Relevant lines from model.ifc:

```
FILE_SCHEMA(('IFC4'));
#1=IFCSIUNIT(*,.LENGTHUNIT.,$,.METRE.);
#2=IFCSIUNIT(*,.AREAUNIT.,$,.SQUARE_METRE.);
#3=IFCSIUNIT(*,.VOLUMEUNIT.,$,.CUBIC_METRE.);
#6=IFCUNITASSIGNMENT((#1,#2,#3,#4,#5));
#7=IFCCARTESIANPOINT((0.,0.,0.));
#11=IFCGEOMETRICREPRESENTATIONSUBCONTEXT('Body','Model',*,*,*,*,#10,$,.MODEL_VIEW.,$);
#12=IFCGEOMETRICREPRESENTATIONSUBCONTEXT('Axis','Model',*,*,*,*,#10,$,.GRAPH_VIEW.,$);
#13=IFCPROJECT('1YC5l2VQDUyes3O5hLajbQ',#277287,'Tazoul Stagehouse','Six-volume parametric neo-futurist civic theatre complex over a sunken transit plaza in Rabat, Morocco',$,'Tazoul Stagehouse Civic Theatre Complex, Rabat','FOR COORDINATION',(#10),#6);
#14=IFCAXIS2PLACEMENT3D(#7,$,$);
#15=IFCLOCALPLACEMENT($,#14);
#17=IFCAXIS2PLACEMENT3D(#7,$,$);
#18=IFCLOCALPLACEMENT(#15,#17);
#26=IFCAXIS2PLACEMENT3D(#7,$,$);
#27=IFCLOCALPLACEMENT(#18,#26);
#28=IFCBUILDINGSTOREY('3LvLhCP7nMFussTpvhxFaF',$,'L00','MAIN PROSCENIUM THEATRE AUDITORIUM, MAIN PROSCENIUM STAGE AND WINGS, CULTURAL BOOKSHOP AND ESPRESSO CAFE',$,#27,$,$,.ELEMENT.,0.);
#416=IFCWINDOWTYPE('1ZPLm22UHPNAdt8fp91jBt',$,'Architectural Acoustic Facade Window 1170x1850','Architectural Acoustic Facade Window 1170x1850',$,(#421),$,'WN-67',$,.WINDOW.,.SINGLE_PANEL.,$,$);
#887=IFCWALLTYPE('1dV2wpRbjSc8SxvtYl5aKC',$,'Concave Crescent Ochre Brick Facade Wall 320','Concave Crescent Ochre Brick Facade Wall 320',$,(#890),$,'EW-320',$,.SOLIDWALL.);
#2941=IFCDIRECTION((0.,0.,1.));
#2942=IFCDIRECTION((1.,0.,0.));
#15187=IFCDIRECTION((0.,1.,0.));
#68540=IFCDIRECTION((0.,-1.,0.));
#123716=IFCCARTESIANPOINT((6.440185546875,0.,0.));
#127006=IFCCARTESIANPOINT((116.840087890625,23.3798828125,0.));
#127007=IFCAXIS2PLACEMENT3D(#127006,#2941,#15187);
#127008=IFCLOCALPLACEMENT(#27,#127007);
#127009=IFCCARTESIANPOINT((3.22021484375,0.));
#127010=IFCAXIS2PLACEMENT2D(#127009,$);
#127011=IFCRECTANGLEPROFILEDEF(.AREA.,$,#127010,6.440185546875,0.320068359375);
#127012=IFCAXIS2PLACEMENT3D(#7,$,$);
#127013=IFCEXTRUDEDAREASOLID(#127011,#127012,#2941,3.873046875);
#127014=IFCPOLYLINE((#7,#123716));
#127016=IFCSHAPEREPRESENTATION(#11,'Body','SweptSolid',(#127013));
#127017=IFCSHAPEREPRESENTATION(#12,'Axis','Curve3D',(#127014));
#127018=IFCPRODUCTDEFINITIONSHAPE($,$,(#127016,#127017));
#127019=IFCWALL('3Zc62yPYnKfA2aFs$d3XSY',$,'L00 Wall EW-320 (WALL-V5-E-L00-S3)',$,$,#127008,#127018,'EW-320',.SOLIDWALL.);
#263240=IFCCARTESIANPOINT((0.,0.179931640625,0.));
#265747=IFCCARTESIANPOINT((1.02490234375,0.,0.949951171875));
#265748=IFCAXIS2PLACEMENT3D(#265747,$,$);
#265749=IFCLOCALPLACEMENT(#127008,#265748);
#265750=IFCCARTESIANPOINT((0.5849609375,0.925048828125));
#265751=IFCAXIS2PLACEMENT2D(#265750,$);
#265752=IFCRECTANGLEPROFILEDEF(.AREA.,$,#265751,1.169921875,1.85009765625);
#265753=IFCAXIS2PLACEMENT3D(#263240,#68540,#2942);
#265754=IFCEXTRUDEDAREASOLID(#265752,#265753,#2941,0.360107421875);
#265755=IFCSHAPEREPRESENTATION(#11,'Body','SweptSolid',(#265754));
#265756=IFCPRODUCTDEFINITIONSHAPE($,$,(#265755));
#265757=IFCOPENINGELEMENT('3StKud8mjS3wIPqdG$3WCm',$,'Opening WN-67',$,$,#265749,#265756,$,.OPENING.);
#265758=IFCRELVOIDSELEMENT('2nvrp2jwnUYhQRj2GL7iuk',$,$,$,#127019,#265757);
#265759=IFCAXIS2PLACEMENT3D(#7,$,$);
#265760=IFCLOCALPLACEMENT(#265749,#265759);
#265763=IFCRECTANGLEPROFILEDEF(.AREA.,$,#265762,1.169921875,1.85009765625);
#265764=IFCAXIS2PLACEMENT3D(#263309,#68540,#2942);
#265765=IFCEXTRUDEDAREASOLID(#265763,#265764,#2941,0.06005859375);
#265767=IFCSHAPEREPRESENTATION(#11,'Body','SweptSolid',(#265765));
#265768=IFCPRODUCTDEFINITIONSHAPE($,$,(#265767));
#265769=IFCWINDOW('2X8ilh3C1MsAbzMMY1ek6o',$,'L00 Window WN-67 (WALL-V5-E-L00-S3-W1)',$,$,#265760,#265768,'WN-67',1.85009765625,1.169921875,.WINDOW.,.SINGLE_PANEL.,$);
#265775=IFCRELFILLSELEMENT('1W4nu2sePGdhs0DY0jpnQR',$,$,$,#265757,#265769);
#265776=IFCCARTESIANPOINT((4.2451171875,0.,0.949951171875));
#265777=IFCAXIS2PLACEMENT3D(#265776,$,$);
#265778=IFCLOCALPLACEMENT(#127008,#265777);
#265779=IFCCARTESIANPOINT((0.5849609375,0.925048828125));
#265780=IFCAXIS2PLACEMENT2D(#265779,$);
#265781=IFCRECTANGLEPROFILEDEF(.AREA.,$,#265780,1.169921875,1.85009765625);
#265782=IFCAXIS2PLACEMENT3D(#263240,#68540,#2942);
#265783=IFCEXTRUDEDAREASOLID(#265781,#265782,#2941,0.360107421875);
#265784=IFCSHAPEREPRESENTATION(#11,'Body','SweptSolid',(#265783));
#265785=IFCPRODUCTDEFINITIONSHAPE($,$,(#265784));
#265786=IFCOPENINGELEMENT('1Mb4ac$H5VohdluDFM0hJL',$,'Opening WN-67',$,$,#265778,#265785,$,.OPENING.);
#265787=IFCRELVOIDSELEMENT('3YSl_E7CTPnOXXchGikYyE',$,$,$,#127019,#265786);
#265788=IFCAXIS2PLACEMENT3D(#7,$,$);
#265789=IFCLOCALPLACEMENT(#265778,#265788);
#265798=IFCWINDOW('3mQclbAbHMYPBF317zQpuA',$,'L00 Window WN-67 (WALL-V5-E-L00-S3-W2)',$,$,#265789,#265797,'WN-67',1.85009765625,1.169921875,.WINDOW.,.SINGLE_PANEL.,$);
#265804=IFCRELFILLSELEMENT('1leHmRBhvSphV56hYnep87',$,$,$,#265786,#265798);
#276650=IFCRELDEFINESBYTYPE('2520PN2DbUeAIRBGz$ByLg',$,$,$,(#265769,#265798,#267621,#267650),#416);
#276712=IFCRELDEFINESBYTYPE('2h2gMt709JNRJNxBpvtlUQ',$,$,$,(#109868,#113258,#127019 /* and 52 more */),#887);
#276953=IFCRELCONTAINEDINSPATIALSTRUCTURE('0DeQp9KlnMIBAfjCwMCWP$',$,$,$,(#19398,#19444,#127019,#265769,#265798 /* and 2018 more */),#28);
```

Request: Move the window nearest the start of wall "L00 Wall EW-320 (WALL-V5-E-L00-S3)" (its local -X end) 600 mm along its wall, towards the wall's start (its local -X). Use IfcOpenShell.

```python
import ifcopenshell
import ifcopenshell.api.geometry
import ifcopenshell.util.placement
import ifcopenshell.util.unit

model = ifcopenshell.open("model.ifc")
unit_scale = ifcopenshell.util.unit.calculate_unit_scale(model)

window = model.by_id(265769)
opening = window.FillsVoids[0].RelatingOpeningElement
wall = opening.VoidsElements[0].RelatingBuildingElement

wall_matrix = ifcopenshell.util.placement.get_local_placement(wall.ObjectPlacement)
shift = wall_matrix[:3, 0] * -0.6 / unit_scale
before = ifcopenshell.util.placement.get_local_placement(window.ObjectPlacement)[:3, 3].copy()

# The window is placed relative to its opening, so it follows when the opening moves.
matrix = ifcopenshell.util.placement.get_local_placement(opening.ObjectPlacement)
matrix[:3, 3] += shift
ifcopenshell.api.geometry.edit_object_placement(
    model, product=opening, matrix=matrix, is_si=False, should_transform_children=True
)

after = ifcopenshell.util.placement.get_local_placement(window.ObjectPlacement)[:3, 3]
print("window moved by", (after - before).round(3) + 0.0)

model.write("model_v2.ifc")
```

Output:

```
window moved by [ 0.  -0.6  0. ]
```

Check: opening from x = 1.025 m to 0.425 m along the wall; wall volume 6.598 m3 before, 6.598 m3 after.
